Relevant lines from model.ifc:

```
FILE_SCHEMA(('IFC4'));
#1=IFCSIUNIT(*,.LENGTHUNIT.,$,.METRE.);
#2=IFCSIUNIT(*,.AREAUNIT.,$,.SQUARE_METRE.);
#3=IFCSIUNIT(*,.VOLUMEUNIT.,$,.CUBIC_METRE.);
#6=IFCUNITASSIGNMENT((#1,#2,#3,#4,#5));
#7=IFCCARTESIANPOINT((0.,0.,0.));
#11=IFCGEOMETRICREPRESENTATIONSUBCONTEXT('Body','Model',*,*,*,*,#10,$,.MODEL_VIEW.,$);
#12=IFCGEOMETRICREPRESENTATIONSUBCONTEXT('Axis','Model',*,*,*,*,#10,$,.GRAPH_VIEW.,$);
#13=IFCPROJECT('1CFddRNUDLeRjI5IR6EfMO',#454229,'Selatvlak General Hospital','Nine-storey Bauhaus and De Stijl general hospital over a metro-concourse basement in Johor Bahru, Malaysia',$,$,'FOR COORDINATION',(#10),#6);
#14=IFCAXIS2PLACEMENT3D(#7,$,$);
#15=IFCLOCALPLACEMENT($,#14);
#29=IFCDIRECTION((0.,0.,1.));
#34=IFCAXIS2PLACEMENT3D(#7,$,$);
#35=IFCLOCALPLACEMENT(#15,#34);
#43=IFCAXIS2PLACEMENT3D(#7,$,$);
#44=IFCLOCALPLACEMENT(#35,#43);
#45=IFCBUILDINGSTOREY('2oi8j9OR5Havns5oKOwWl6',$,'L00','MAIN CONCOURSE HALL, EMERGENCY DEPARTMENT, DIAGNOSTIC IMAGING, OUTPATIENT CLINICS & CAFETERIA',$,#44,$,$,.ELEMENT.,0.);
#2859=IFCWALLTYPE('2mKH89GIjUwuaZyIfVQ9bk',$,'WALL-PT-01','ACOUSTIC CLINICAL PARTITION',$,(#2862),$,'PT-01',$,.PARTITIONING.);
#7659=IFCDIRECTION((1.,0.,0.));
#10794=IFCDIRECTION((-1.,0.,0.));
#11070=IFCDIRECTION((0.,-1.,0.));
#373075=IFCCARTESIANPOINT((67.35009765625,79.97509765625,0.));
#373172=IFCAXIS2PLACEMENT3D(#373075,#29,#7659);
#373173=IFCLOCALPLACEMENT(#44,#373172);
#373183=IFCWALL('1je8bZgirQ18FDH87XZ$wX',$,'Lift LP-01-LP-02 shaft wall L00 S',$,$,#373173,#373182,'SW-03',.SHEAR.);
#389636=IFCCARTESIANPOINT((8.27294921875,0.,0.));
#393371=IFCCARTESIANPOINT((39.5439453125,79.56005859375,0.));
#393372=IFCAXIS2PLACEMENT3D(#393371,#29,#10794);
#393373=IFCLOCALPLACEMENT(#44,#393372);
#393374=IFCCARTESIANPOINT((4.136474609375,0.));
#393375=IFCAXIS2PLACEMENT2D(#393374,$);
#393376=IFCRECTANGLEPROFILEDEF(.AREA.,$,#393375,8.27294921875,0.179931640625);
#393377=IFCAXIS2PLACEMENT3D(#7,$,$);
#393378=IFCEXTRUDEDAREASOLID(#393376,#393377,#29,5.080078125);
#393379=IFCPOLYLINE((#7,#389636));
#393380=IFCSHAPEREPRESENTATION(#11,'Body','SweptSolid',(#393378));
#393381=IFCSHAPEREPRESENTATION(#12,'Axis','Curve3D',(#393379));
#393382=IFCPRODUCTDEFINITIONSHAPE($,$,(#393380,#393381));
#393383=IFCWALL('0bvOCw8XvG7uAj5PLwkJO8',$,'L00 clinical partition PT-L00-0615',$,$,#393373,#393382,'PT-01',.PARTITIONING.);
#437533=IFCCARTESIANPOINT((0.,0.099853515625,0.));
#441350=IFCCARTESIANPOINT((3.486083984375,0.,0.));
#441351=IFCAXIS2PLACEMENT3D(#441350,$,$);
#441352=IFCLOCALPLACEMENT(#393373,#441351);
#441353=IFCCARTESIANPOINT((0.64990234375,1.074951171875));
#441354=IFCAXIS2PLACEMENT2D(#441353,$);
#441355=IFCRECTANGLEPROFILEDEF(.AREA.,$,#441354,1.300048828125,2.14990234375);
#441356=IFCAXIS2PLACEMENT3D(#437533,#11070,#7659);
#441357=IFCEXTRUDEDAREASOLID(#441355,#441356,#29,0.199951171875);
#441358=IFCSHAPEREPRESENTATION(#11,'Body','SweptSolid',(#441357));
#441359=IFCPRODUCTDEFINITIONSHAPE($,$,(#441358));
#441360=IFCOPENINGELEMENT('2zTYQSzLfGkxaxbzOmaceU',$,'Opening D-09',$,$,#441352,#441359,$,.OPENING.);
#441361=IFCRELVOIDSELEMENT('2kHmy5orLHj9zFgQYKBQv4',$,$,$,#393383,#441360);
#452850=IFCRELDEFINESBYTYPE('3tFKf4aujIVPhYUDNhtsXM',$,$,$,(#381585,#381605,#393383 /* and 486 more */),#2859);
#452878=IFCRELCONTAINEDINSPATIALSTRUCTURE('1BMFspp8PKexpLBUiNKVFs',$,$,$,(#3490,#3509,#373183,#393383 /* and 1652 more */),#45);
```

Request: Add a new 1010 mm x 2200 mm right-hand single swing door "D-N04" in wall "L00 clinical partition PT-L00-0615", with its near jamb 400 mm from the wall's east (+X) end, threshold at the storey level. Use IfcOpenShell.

```python
import numpy as np
import ifcopenshell
import ifcopenshell.api.feature
import ifcopenshell.api.geometry
import ifcopenshell.api.root
import ifcopenshell.api.spatial
import ifcopenshell.geom
import ifcopenshell.util.element
import ifcopenshell.util.placement
import ifcopenshell.util.representation
import ifcopenshell.util.shape
import ifcopenshell.util.unit

model = ifcopenshell.open("model.ifc")
unit_scale = ifcopenshell.util.unit.calculate_unit_scale(model)
settings = ifcopenshell.geom.settings()


def volume(element):
    """Net volume in cubic metres, openings subtracted."""
    shape = ifcopenshell.geom.create_shape(settings, element)
    return ifcopenshell.util.shape.get_volume(shape.geometry)


wall = model.by_guid("0bvOCw8XvG7uAj5PLwkJO8")
storey = ifcopenshell.util.element.get_container(wall, ifc_class="IfcBuildingStorey")
context = ifcopenshell.util.representation.get_context(model, "Model", "Body", "MODEL_VIEW")
before = volume(wall)

width, height, from_end, sill = 1.01, 2.2, 0.4, 0.0  # metres

# The wall runs along its own X axis, and the end named is its -X end.
wall_shape = ifcopenshell.geom.create_shape(settings, wall)
x, y, z = ifcopenshell.util.shape.get_vertices(wall_shape.geometry).T
start = x.min() + from_end
face, thickness = float(y.min()), float(y.max() - y.min())
wall_matrix = ifcopenshell.util.placement.get_local_placement(wall.ObjectPlacement)
level = ifcopenshell.util.placement.get_local_placement(storey.ObjectPlacement)[2, 3]


def in_wall(x, y):
    """Placement at x, y metres in the wall's axes, at sill height."""
    matrix = wall_matrix.copy()
    matrix[:, 3] = wall_matrix @ np.array([x / unit_scale, y / unit_scale, 0.0, 1.0])
    matrix[2, 3] = level + sill / unit_scale
    return matrix


# Opening: a box that overshoots both wall faces by 50 mm.
opening = ifcopenshell.api.root.create_entity(model, ifc_class="IfcOpeningElement", predefined_type="OPENING")
box = ifcopenshell.api.geometry.add_wall_representation(
    model, context=context, length=width, height=height, thickness=thickness + 0.1
)
ifcopenshell.api.geometry.assign_representation(model, product=opening, representation=box)
ifcopenshell.api.geometry.edit_object_placement(model, product=opening, matrix=in_wall(start, face - 0.05), is_si=False)
ifcopenshell.api.feature.add_feature(model, feature=opening, element=wall)

door = ifcopenshell.api.root.create_entity(model, ifc_class="IfcDoor", name="D-N04", predefined_type="DOOR")
door.OverallWidth, door.OverallHeight = width / unit_scale, height / unit_scale
door.OperationType = "SINGLE_SWING_RIGHT"
body = ifcopenshell.api.geometry.add_door_representation(
    model,
    context=context,
    overall_width=door.OverallWidth,
    overall_height=door.OverallHeight,
    operation_type="SINGLE_SWING_RIGHT",
    lining_properties={"LiningDepth": thickness / unit_scale, "ThresholdDepth": thickness / unit_scale},
)
ifcopenshell.api.geometry.assign_representation(model, product=door, representation=body)
ifcopenshell.api.spatial.assign_container(model, products=[door], relating_structure=storey)
ifcopenshell.api.feature.add_filling(model, opening=opening, element=door)

# The lining spans the wall, so the door starts at the wall face.
ifcopenshell.api.geometry.edit_object_placement(model, product=door, matrix=in_wall(start, face), is_si=False)

after = volume(wall)

print(f"wall volume {before:.3f} -> {after:.3f} m3")

model.write("model_rev.ifc")
```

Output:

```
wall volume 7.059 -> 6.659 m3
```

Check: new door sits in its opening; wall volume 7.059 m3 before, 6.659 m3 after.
